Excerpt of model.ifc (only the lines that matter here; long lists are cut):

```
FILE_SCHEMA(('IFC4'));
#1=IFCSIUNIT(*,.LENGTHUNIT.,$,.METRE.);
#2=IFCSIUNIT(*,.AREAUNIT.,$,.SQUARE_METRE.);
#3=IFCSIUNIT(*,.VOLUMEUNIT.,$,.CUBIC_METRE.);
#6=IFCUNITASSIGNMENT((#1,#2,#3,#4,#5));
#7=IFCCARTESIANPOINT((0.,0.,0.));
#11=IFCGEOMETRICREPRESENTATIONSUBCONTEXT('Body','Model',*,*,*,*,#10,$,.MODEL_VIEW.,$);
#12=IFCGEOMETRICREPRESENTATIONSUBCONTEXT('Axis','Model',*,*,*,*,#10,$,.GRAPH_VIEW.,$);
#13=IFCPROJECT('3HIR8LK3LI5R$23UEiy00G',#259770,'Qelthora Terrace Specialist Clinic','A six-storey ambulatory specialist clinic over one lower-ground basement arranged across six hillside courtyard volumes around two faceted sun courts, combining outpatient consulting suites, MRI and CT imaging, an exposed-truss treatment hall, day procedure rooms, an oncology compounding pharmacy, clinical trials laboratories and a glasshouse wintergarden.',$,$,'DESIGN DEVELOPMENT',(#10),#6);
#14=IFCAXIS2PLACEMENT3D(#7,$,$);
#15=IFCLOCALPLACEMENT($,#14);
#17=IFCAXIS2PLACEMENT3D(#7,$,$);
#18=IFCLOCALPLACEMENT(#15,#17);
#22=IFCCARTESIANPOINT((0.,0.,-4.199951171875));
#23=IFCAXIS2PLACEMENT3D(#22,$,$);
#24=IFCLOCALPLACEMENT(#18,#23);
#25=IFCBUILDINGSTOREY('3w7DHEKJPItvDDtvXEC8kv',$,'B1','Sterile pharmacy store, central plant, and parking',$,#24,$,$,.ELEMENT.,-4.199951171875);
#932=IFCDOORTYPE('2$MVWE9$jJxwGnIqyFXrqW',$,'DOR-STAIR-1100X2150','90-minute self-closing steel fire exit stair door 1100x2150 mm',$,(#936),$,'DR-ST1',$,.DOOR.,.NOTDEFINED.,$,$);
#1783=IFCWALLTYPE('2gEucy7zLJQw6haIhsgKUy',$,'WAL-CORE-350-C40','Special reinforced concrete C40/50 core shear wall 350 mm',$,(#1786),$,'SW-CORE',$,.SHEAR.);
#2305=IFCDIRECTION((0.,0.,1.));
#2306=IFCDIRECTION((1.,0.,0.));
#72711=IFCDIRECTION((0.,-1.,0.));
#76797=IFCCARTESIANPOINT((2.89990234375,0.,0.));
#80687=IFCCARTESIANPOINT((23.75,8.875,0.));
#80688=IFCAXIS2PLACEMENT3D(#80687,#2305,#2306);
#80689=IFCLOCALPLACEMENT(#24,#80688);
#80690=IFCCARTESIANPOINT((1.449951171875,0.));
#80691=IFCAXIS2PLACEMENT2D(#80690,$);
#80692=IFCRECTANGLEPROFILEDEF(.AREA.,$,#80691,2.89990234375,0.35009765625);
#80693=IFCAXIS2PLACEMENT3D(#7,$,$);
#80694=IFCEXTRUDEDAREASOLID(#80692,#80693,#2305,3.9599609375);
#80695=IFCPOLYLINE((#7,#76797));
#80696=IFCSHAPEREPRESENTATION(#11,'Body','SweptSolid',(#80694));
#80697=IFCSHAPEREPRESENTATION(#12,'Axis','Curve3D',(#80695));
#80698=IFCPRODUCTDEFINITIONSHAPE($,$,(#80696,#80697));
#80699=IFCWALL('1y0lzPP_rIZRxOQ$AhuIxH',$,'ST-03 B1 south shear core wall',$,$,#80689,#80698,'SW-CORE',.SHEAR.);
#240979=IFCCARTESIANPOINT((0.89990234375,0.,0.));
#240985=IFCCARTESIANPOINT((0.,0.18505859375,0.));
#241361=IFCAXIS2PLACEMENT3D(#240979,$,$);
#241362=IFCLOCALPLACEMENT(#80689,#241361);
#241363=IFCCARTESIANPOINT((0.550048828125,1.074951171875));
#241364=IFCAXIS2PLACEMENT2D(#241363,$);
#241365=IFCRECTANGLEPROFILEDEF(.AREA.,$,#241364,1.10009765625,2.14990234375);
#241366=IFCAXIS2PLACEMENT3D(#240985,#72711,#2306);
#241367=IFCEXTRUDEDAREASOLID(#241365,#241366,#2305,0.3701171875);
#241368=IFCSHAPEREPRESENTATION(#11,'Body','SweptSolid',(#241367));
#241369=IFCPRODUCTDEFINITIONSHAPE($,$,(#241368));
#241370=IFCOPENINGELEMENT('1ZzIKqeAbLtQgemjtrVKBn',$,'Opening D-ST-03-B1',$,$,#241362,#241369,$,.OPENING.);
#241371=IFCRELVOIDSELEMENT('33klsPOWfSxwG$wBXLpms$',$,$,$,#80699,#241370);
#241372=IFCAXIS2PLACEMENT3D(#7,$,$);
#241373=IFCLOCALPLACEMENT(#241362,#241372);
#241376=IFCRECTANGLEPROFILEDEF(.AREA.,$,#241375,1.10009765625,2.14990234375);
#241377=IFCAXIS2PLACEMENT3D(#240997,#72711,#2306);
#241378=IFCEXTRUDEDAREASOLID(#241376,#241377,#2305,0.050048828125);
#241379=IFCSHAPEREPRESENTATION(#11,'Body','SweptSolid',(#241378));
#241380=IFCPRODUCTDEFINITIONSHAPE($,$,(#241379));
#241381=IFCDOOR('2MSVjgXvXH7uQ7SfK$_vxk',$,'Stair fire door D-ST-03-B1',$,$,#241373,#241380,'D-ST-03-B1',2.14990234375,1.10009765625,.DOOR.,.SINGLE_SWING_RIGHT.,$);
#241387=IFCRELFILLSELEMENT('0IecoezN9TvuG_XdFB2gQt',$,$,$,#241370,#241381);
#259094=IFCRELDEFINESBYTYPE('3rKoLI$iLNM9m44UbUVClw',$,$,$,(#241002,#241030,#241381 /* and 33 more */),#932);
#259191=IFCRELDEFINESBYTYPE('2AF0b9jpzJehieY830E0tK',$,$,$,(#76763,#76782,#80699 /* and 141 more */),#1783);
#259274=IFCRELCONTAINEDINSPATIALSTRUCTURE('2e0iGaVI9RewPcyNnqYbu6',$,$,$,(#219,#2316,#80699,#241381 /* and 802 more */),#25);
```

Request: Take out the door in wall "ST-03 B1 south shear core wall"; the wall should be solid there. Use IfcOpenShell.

```python
import ifcopenshell
import ifcopenshell.api.feature
import ifcopenshell.api.root
import ifcopenshell.geom
import ifcopenshell.util.shape

model = ifcopenshell.open("model.ifc")
settings = ifcopenshell.geom.settings()


def volume(element):
    """Net volume in cubic metres, openings subtracted."""
    shape = ifcopenshell.geom.create_shape(settings, element)
    return ifcopenshell.util.shape.get_volume(shape.geometry)


door = model.by_guid("2MSVjgXvXH7uQ7SfK$_vxk")
opening = door.FillsVoids[0].RelatingOpeningElement
wall = opening.VoidsElements[0].RelatingBuildingElement
before = volume(wall)

ifcopenshell.api.root.remove_product(model, product=door)
ifcopenshell.api.feature.remove_feature(model, feature=opening)

after = volume(wall)

print(f"wall volume {before:.3f} -> {after:.3f} m3")

model.write("model-out.ifc")
```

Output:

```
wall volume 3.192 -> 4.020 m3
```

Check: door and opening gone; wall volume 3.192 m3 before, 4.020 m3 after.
